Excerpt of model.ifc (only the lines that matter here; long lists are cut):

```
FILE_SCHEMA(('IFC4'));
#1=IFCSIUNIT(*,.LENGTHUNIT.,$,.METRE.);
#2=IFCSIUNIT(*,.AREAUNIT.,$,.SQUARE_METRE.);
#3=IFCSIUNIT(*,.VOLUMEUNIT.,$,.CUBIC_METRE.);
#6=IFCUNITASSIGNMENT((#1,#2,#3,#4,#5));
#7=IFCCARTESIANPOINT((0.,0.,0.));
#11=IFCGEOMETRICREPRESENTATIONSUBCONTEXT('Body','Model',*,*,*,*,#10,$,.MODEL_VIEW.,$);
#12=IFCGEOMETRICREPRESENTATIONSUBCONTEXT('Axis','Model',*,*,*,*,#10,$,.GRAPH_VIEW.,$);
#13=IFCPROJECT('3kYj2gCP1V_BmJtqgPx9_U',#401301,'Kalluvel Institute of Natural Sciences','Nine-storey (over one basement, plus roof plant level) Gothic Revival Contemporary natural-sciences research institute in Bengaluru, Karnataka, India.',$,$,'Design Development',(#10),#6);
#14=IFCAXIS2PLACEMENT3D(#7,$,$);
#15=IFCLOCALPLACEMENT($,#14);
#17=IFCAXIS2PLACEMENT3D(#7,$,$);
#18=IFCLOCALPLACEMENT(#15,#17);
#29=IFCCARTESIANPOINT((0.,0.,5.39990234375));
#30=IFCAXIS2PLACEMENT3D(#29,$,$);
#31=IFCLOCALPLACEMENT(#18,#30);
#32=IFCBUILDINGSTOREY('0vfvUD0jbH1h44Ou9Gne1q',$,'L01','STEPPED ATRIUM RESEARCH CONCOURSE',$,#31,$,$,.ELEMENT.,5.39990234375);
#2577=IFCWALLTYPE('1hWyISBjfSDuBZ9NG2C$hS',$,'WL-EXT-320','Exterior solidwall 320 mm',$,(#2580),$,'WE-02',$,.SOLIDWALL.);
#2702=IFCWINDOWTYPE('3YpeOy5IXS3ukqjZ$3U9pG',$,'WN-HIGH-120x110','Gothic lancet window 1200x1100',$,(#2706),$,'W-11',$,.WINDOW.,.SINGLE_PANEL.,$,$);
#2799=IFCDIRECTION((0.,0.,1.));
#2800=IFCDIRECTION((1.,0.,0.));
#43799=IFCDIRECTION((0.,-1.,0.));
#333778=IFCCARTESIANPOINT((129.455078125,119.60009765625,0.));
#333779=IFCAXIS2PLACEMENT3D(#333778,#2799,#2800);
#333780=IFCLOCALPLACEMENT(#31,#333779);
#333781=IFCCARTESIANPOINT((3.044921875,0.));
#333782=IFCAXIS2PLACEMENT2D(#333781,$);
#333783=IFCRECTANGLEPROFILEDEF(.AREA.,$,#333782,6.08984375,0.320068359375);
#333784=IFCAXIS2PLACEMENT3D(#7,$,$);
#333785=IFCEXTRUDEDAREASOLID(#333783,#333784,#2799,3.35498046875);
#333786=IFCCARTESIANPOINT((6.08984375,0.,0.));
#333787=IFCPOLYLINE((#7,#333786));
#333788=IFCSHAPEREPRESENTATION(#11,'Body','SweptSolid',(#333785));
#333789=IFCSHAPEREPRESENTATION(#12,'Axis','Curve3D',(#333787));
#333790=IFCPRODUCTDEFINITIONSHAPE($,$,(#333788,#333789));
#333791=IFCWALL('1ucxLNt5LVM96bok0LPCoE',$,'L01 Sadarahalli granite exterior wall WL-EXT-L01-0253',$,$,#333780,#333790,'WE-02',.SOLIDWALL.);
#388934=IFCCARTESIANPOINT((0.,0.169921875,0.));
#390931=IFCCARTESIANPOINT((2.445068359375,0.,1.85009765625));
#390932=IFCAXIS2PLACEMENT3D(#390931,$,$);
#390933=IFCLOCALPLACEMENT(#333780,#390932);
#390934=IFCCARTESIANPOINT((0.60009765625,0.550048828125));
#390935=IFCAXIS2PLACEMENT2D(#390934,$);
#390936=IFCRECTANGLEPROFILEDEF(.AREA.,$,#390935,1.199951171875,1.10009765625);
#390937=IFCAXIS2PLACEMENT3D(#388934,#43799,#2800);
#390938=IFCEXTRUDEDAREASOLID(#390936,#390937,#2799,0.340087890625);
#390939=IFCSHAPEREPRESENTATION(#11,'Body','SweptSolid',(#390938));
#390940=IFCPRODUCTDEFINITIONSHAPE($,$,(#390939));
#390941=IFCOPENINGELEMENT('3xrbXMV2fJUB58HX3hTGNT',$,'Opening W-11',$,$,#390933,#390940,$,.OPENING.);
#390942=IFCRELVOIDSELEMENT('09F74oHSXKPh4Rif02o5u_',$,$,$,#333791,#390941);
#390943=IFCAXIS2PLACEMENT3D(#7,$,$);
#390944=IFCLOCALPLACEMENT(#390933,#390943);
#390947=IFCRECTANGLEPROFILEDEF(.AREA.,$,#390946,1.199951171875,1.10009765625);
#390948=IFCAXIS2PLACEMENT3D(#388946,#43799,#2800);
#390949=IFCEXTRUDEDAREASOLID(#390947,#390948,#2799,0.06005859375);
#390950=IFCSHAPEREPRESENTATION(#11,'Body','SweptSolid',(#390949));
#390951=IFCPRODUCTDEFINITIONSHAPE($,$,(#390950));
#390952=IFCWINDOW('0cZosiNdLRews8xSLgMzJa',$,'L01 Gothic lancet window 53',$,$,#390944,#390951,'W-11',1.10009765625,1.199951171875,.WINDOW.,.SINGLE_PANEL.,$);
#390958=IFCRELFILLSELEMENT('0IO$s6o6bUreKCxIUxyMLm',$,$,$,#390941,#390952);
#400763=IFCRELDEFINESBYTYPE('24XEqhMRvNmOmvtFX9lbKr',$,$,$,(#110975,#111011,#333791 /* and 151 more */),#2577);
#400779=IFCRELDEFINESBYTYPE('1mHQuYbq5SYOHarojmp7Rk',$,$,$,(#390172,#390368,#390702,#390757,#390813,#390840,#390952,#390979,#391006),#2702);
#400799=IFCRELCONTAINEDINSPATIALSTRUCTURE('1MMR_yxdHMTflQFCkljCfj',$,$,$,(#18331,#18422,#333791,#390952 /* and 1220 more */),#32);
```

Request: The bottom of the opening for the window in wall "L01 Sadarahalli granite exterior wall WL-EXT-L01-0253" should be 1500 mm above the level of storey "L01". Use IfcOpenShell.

```python
import numpy as np
import ifcopenshell
import ifcopenshell.api.geometry
import ifcopenshell.geom
import ifcopenshell.util.element
import ifcopenshell.util.placement
import ifcopenshell.util.shape
import ifcopenshell.util.unit

model = ifcopenshell.open("model.ifc")
unit_scale = ifcopenshell.util.unit.calculate_unit_scale(model)

window = model.by_guid("0cZosiNdLRews8xSLgMzJa")
opening = window.FillsVoids[0].RelatingOpeningElement
storey = ifcopenshell.util.element.get_container(window, ifc_class="IfcBuildingStorey")
level = ifcopenshell.util.placement.get_local_placement(storey.ObjectPlacement)[2, 3]

# The opening's origin need not be at the sill, so measure its lowest point.
shape = ifcopenshell.geom.create_shape(ifcopenshell.geom.settings(), opening)
bottom = ifcopenshell.util.shape.get_shape_bottom_elevation(shape, shape.geometry) / unit_scale
dz = level + 1.5 - bottom

shift = np.array([0.0, 0.0, dz])
# The window is placed relative to its opening, so it follows when the opening moves.
matrix = ifcopenshell.util.placement.get_local_placement(opening.ObjectPlacement)
matrix[:3, 3] += shift
ifcopenshell.api.geometry.edit_object_placement(
    model, product=opening, matrix=matrix, is_si=False, should_transform_children=True
)

print(f"moved by {dz * unit_scale:+.3f} m")

model.write("model-out.ifc")
```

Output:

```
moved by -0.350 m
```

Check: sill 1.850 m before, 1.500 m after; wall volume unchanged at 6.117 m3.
